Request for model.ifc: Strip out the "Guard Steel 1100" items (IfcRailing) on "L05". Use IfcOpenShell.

First a look at what the model holds.

```python
import ifcopenshell
import ifcopenshell.util.element

model = ifcopenshell.open("model.ifc")
print(model.schema)
storey = next(s for s in model.by_type("IfcBuildingStorey") if s.Name == "L05")
railings = [e for e in ifcopenshell.util.element.get_decomposition(storey) if e.is_a("IfcRailing")]
seen = {}
for e in railings:
    element_type = ifcopenshell.util.element.get_type(e)
    name = element_type.Name if element_type not in (None, e) else None
    seen[name] = seen.get(name, 0) + 1
for name, count in sorted(seen.items(), key=str):
    print(count, "x", name)
```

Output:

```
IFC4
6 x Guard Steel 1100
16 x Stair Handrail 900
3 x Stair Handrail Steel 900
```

```python
import ifcopenshell
import ifcopenshell.api.root
import ifcopenshell.util.element

model = ifcopenshell.open("model.ifc")

storey = next(s for s in model.by_type("IfcBuildingStorey") if s.Name == "L05")
railings = [e for e in ifcopenshell.util.element.get_decomposition(storey) if e.is_a("IfcRailing")]
targets = [e for e in railings if (t := ifcopenshell.util.element.get_type(e)) not in (None, e) and t.Name == "Guard Steel 1100"]

for e in targets:
    ifcopenshell.api.root.remove_product(model, product=e)
print(len(targets), "removed")

model.write("model_v2.ifc")
```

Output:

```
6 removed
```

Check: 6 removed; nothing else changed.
